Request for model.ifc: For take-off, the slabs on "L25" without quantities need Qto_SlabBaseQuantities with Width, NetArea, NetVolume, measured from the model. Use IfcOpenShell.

First a look at what the model holds.

```python
import ifcopenshell
import ifcopenshell.util.element
import ifcopenshell.util.unit

model = ifcopenshell.open("model.ifc")
print(model.schema)
for unit_type in ("LENGTHUNIT", "AREAUNIT", "VOLUMEUNIT"):
    print(unit_type, ifcopenshell.util.unit.calculate_unit_scale(model, unit_type))
storey = next(s for s in model.by_type("IfcBuildingStorey") if s.Name == "L25")
slabs = [e for e in ifcopenshell.util.element.get_decomposition(storey) if e.is_a("IfcSlab")]
for e in sorted(slabs, key=lambda e: e.id()):
    print(e.id(), e.is_a(), e.Name, list(ifcopenshell.util.element.get_psets(e, qtos_only=True)), sep=" | ")
```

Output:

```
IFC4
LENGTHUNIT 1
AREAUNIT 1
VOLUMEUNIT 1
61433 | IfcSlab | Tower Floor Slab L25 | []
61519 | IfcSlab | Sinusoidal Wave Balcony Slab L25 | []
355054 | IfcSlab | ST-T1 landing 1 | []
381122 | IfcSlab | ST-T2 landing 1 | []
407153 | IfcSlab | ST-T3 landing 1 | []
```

```python
import ifcopenshell
import ifcopenshell.api.pset
import ifcopenshell.geom
import ifcopenshell.util.element
import ifcopenshell.util.shape
import ifcopenshell.util.unit

model = ifcopenshell.open("model.ifc")
unit_scale = ifcopenshell.util.unit.calculate_unit_scale(model)
area_scale = ifcopenshell.util.unit.calculate_unit_scale(model, "AREAUNIT")
volume_scale = ifcopenshell.util.unit.calculate_unit_scale(model, "VOLUMEUNIT")
settings = ifcopenshell.geom.settings()

storey = next(s for s in model.by_type("IfcBuildingStorey") if s.Name == "L25")
slabs = [e for e in ifcopenshell.util.element.get_decomposition(storey) if e.is_a("IfcSlab")]

for e in sorted(slabs, key=lambda e: e.id()):
    if ifcopenshell.util.element.get_psets(e, qtos_only=True, should_inherit=False):
        continue
    # Geometry comes back in metres, in the element's own axes.
    shape = ifcopenshell.geom.create_shape(settings, e)
    values = {
        "Width": ifcopenshell.util.shape.get_z(shape.geometry) / unit_scale,
        "NetArea": ifcopenshell.util.shape.get_footprint_area(shape.geometry) / area_scale,
        "NetVolume": ifcopenshell.util.shape.get_volume(shape.geometry) / volume_scale,
    }
    qto = ifcopenshell.api.pset.add_qto(model, product=e, name="Qto_SlabBaseQuantities")
    ifcopenshell.api.pset.edit_qto(model, qto=qto, properties=values)
    print(e.id(), {k: round(v, 3) for k, v in values.items()})

model.write("model_rev.ifc")
```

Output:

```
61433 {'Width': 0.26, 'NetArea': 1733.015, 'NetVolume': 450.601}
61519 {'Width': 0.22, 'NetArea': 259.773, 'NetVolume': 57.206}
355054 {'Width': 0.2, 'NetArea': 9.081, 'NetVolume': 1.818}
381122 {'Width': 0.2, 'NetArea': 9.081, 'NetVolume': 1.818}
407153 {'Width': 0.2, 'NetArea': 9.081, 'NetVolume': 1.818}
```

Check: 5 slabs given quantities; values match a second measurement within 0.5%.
